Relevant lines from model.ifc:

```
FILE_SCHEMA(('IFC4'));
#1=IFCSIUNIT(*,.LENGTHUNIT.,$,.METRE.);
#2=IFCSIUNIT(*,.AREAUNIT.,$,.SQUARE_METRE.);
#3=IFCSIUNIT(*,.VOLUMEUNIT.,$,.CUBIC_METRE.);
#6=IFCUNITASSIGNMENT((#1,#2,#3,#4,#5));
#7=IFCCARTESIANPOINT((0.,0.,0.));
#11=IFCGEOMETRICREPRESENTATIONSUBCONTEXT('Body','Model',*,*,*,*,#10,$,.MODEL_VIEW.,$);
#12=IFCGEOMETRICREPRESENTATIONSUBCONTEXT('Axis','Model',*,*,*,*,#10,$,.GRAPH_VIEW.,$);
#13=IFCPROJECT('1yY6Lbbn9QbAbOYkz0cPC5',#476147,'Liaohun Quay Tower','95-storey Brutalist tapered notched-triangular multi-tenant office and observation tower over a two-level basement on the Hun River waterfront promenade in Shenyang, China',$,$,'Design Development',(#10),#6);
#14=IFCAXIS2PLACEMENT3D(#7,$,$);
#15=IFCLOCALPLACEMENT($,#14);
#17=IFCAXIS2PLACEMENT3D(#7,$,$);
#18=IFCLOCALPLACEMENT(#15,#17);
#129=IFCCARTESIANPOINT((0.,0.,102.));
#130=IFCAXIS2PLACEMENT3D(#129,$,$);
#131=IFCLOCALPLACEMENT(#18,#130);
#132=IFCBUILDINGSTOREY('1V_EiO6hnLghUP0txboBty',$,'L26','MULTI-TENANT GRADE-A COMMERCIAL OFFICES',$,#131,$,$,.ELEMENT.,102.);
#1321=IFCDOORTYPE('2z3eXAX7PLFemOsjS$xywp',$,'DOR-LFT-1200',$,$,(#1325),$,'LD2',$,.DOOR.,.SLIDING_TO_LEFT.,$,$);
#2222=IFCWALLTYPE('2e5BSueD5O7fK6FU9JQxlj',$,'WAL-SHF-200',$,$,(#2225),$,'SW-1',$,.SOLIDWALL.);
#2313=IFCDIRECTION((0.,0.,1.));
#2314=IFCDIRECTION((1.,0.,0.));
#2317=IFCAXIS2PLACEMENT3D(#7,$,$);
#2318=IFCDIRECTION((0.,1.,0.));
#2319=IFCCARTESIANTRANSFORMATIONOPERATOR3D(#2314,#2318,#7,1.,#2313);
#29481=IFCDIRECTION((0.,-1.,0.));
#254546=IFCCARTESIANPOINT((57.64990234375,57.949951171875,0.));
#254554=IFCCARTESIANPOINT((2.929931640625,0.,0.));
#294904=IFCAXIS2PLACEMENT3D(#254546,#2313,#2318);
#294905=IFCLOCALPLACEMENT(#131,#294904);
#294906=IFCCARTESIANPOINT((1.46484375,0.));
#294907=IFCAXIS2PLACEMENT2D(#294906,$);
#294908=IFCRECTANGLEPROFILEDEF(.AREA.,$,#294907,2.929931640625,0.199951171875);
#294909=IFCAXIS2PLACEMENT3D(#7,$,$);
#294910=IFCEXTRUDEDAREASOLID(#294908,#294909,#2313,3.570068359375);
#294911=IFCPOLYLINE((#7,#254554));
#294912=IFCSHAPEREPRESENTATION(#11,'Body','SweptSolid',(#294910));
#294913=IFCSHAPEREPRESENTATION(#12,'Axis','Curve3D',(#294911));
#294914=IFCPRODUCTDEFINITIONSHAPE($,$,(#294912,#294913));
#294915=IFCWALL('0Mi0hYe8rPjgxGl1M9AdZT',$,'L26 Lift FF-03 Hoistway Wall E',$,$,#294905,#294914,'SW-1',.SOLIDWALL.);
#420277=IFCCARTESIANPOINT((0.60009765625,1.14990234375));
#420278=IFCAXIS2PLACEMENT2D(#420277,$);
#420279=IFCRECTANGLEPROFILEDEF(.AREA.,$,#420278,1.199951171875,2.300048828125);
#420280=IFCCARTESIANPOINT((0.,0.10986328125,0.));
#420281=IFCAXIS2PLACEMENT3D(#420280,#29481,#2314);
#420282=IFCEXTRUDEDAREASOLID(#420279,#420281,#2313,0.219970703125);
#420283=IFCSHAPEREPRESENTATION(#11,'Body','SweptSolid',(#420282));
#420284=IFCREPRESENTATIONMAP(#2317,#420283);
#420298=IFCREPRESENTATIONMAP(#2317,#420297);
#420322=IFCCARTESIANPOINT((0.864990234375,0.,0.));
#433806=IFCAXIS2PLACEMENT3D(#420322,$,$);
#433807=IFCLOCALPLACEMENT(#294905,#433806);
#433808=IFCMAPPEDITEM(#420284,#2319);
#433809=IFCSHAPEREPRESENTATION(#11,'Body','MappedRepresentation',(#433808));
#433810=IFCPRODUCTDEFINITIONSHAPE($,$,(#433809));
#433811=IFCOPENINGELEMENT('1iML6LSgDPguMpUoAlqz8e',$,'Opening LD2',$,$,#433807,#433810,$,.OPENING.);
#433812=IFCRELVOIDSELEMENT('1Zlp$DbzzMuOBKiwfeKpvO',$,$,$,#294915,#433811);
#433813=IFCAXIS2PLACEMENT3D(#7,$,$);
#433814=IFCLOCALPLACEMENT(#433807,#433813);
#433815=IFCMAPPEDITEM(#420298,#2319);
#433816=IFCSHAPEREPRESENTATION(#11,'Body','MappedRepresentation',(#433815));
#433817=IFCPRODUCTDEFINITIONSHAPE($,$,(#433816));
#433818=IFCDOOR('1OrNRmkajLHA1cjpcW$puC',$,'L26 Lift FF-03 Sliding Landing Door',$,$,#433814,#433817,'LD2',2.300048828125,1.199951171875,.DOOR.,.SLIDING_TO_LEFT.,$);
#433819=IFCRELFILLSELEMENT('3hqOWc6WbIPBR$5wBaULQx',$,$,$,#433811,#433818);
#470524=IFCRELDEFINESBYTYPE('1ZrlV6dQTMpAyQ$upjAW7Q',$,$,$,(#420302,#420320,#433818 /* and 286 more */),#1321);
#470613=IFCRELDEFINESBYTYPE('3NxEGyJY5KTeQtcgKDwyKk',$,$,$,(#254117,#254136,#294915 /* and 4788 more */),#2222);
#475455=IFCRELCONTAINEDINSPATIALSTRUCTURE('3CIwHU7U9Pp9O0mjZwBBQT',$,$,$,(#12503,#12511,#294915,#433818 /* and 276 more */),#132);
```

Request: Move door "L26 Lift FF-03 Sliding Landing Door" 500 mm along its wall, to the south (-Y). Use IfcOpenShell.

```python
import ifcopenshell
import ifcopenshell.api.geometry
import ifcopenshell.util.placement

model = ifcopenshell.open("model.ifc")

door = model.by_id(433818)
opening = door.FillsVoids[0].RelatingOpeningElement
wall = opening.VoidsElements[0].RelatingBuildingElement

wall_matrix = ifcopenshell.util.placement.get_local_placement(wall.ObjectPlacement)
shift = wall_matrix[:3, 0] * -0.5
before = ifcopenshell.util.placement.get_local_placement(door.ObjectPlacement)[:3, 3].copy()

# The door is placed relative to its opening, so it follows when the opening moves.
matrix = ifcopenshell.util.placement.get_local_placement(opening.ObjectPlacement)
matrix[:3, 3] += shift
ifcopenshell.api.geometry.edit_object_placement(
    model, product=opening, matrix=matrix, is_si=False, should_transform_children=True
)

after = ifcopenshell.util.placement.get_local_placement(door.ObjectPlacement)[:3, 3]
print("door moved by", (after - before).round(3) + 0.0)

model.write("model_updated.ifc")
```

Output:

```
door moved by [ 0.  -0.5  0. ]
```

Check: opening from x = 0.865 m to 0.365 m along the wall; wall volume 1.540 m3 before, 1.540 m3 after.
